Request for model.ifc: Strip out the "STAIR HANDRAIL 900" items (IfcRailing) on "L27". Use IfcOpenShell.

First a look at what the model holds.

```python
import ifcopenshell
import ifcopenshell.util.element

model = ifcopenshell.open("model.ifc")
print(model.schema)
storey = next(s for s in model.by_type("IfcBuildingStorey") if s.Name == "L27")
railings = [e for e in ifcopenshell.util.element.get_decomposition(storey) if e.is_a("IfcRailing")]
seen = {}
for e in railings:
    element_type = ifcopenshell.util.element.get_type(e)
    name = element_type.Name if element_type not in (None, e) else None
    seen[name] = seen.get(name, 0) + 1
for name, count in sorted(seen.items(), key=str):
    print(count, "x", name)
```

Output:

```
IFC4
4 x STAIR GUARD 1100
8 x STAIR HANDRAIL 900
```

```python
import ifcopenshell
import ifcopenshell.api.root
import ifcopenshell.util.element

model = ifcopenshell.open("model.ifc")

storey = next(s for s in model.by_type("IfcBuildingStorey") if s.Name == "L27")
railings = [e for e in ifcopenshell.util.element.get_decomposition(storey) if e.is_a("IfcRailing")]
targets = [e for e in railings if (t := ifcopenshell.util.element.get_type(e)) not in (None, e) and t.Name == "STAIR HANDRAIL 900"]

for e in targets:
    ifcopenshell.api.root.remove_product(model, product=e)
print(len(targets), "removed")

model.write("model_edited.ifc")
```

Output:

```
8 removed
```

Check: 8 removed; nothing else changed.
